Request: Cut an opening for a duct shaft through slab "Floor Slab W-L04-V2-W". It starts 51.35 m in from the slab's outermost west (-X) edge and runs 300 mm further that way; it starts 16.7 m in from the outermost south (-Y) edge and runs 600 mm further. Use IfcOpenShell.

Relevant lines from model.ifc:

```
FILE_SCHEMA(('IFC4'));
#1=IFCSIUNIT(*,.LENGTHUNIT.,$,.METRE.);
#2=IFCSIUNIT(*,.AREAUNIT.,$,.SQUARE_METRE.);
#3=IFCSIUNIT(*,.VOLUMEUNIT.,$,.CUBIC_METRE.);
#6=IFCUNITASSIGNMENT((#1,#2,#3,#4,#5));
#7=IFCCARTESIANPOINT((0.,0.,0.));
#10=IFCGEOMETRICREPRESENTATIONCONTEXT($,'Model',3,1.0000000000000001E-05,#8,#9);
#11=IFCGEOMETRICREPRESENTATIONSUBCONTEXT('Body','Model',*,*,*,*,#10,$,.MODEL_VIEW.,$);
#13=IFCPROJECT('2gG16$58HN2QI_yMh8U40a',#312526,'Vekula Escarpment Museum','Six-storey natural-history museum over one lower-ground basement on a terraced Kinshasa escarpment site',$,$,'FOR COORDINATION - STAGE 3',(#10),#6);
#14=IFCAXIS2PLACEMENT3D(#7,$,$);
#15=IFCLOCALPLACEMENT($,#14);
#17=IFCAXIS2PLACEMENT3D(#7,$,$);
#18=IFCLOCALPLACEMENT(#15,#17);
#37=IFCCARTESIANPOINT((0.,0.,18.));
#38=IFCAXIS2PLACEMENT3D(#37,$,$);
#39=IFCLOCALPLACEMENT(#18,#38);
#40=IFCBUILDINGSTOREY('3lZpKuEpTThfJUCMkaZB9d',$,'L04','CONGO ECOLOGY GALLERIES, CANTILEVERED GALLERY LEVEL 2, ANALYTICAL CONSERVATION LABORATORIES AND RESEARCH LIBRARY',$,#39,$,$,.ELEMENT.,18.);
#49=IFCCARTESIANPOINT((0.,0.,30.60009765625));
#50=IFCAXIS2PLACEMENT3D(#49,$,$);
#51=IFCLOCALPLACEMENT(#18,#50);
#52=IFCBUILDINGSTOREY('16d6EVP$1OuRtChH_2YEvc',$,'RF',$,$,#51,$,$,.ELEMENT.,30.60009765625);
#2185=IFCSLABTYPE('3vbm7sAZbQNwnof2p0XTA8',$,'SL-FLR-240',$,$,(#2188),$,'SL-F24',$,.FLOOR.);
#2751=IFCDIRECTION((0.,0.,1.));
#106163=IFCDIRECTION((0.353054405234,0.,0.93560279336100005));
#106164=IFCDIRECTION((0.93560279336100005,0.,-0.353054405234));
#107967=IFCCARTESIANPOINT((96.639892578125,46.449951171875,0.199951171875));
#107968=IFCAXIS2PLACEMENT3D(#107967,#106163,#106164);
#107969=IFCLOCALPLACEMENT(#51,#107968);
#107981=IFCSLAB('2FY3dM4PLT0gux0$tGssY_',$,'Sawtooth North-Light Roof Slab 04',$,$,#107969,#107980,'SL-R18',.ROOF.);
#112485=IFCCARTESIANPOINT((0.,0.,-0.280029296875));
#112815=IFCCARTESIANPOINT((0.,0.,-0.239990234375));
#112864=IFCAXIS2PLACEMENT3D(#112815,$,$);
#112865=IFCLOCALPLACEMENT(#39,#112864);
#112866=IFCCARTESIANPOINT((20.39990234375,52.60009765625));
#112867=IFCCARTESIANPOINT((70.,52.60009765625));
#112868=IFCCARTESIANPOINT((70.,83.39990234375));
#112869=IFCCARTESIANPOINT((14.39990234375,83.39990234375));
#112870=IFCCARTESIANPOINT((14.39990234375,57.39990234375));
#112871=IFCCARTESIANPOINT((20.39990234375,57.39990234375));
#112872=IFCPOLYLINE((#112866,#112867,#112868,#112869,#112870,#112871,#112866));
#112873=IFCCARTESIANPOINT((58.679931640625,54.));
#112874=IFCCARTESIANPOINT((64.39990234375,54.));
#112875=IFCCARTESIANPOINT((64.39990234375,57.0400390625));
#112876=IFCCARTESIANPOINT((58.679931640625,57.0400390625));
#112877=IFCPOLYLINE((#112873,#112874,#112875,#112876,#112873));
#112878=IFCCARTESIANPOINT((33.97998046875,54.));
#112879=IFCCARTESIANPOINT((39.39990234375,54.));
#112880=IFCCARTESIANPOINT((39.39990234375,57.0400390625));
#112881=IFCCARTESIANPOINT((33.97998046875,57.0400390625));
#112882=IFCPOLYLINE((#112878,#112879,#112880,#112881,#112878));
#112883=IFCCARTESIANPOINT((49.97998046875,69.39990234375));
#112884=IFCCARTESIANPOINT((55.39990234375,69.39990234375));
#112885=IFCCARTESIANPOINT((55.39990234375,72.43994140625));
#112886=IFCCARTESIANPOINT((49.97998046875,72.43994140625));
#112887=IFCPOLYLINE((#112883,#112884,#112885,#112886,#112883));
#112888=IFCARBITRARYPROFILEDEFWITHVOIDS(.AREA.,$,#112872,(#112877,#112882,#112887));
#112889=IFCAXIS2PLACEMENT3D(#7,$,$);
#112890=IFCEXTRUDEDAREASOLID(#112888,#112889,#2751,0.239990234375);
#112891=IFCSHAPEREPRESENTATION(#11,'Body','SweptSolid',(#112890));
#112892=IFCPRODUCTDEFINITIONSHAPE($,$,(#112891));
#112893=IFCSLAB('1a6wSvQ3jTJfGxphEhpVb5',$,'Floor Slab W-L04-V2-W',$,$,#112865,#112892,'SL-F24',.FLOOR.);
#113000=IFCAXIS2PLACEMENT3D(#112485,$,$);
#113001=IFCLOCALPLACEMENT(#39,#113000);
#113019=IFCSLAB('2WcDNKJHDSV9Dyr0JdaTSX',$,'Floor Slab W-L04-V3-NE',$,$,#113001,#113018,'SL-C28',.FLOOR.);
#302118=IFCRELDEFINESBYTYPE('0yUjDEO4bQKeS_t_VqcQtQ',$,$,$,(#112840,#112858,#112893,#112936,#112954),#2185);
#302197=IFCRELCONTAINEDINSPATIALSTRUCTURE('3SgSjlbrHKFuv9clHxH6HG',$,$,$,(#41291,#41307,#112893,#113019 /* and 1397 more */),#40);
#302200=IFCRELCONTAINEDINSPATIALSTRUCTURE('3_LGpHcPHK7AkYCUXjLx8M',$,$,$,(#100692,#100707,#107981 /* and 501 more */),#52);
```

```python
import numpy as np
import ifcopenshell
import ifcopenshell.api.feature
import ifcopenshell.api.geometry
import ifcopenshell.api.root
import ifcopenshell.geom
import ifcopenshell.util.placement
import ifcopenshell.util.representation
import ifcopenshell.util.shape
import ifcopenshell.util.unit

model = ifcopenshell.open("model.ifc")
unit_scale = ifcopenshell.util.unit.calculate_unit_scale(model)
settings = ifcopenshell.geom.settings()


def volume(element):
    """Net volume in cubic metres, openings subtracted."""
    shape = ifcopenshell.geom.create_shape(settings, element)
    return ifcopenshell.util.shape.get_volume(shape.geometry)


slab = model.by_id(112893)
before = volume(slab)

# Extent in the slab's own axes, in metres. The edges named are its -X and -Y sides.
slab_shape = ifcopenshell.geom.create_shape(settings, slab)
vertices = ifcopenshell.util.shape.get_vertices(slab_shape.geometry)
x_min, y_min, bottom = vertices.min(axis=0)
top = vertices[:, 2].max()

opening = ifcopenshell.api.root.create_entity(model, ifc_class="IfcOpeningElement", name="Duct shaft opening", predefined_type="OPENING")
context = ifcopenshell.util.representation.get_context(model, "Model", "Body", "MODEL_VIEW")
width, depth = 0.3, 0.6
outline = [(0.0, 0.0), (width, 0.0), (width, depth), (0.0, depth), (0.0, 0.0)]
# Overshoot both faces by 50 mm so the cut is clean.
shape = ifcopenshell.api.geometry.add_slab_representation(
    model, context=context, depth=top - bottom + 0.1, polyline=outline
)
ifcopenshell.api.geometry.assign_representation(model, product=opening, representation=shape)

matrix = ifcopenshell.util.placement.get_local_placement(slab.ObjectPlacement)
matrix[:, 3] = matrix @ np.append(np.array([x_min + 51.35, y_min + 16.7, bottom - 0.05]) / unit_scale, 1.0)
ifcopenshell.api.geometry.edit_object_placement(model, product=opening, matrix=matrix, is_si=False)
ifcopenshell.api.feature.add_feature(model, feature=opening, element=slab)

after = volume(slab)

print(f"slab volume {before:.3f} -> {after:.3f} m3")

model.write("model_v2.ifc")
```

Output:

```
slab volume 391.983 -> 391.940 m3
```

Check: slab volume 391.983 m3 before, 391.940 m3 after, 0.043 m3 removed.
